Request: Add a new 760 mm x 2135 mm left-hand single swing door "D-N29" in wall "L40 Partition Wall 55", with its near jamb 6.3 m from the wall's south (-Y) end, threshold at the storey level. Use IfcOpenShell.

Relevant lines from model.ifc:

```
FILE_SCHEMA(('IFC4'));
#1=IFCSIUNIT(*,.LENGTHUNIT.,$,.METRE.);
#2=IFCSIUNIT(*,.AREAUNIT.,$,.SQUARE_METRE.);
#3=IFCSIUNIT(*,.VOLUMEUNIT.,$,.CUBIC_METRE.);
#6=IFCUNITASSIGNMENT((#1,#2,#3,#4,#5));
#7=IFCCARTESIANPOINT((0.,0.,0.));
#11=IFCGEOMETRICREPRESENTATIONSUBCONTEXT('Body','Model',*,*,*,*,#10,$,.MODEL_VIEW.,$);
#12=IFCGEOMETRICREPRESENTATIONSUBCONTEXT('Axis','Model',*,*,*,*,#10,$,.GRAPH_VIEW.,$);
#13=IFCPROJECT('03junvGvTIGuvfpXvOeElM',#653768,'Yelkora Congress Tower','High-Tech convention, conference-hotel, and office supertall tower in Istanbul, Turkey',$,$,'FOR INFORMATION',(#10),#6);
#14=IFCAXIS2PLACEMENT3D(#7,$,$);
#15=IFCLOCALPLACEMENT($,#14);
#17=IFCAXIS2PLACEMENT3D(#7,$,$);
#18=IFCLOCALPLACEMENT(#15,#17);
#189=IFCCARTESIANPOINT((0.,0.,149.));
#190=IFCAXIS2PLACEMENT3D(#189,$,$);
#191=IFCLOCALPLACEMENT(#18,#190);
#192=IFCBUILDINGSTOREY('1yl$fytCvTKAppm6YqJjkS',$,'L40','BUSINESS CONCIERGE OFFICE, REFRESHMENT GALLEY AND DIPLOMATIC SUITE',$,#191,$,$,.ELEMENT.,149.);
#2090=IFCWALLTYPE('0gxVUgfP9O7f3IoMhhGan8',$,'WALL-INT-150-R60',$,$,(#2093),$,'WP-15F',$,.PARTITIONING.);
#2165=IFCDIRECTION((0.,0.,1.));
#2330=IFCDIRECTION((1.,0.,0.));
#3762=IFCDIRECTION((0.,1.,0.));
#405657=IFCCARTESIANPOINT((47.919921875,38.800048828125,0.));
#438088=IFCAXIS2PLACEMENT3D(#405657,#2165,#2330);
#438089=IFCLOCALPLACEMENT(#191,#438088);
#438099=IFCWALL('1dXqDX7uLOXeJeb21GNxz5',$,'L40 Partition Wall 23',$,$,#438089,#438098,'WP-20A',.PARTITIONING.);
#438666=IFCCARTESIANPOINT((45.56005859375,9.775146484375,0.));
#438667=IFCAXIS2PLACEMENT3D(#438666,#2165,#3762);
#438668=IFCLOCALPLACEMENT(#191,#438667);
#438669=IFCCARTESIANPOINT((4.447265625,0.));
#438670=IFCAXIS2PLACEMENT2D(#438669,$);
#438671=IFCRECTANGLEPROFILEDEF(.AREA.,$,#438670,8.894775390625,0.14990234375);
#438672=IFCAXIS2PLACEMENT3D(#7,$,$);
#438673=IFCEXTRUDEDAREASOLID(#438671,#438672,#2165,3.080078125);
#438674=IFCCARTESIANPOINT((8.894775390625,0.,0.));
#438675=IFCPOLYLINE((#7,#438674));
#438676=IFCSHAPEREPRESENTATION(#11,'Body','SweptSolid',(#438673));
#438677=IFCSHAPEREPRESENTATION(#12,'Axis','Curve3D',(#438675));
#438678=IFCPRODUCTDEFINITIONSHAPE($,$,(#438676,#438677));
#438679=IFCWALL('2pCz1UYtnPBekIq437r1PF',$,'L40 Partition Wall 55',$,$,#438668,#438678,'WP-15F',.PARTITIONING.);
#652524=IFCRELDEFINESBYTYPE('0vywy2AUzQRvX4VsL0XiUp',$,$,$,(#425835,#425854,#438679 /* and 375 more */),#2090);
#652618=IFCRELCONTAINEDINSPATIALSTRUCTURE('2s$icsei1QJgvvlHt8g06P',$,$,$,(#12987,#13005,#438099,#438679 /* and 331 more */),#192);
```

```python
import numpy as np
import ifcopenshell
import ifcopenshell.api.feature
import ifcopenshell.api.geometry
import ifcopenshell.api.root
import ifcopenshell.api.spatial
import ifcopenshell.geom
import ifcopenshell.util.element
import ifcopenshell.util.placement
import ifcopenshell.util.representation
import ifcopenshell.util.shape
import ifcopenshell.util.unit

model = ifcopenshell.open("model.ifc")
unit_scale = ifcopenshell.util.unit.calculate_unit_scale(model)
settings = ifcopenshell.geom.settings()


def volume(element):
    """Net volume in cubic metres, openings subtracted."""
    shape = ifcopenshell.geom.create_shape(settings, element)
    return ifcopenshell.util.shape.get_volume(shape.geometry)


wall = model.by_guid("2pCz1UYtnPBekIq437r1PF")
storey = ifcopenshell.util.element.get_container(wall, ifc_class="IfcBuildingStorey")
context = ifcopenshell.util.representation.get_context(model, "Model", "Body", "MODEL_VIEW")
before = volume(wall)

width, height, from_end, sill = 0.76, 2.135, 6.3, 0.0  # metres

# The wall runs along its own X axis, and the end named is its -X end.
wall_shape = ifcopenshell.geom.create_shape(settings, wall)
x, y, z = ifcopenshell.util.shape.get_vertices(wall_shape.geometry).T
start = x.min() + from_end
face, thickness = float(y.min()), float(y.max() - y.min())
wall_matrix = ifcopenshell.util.placement.get_local_placement(wall.ObjectPlacement)
level = ifcopenshell.util.placement.get_local_placement(storey.ObjectPlacement)[2, 3]


def in_wall(x, y):
    """Placement at x, y metres in the wall's axes, at sill height."""
    matrix = wall_matrix.copy()
    matrix[:, 3] = wall_matrix @ np.array([x / unit_scale, y / unit_scale, 0.0, 1.0])
    matrix[2, 3] = level + sill / unit_scale
    return matrix


# Opening: a box that overshoots both wall faces by 50 mm.
opening = ifcopenshell.api.root.create_entity(model, ifc_class="IfcOpeningElement", predefined_type="OPENING")
box = ifcopenshell.api.geometry.add_wall_representation(
    model, context=context, length=width, height=height, thickness=thickness + 0.1
)
ifcopenshell.api.geometry.assign_representation(model, product=opening, representation=box)
ifcopenshell.api.geometry.edit_object_placement(model, product=opening, matrix=in_wall(start, face - 0.05), is_si=False)
ifcopenshell.api.feature.add_feature(model, feature=opening, element=wall)

door = ifcopenshell.api.root.create_entity(model, ifc_class="IfcDoor", name="D-N29", predefined_type="DOOR")
door.OverallWidth, door.OverallHeight = width / unit_scale, height / unit_scale
door.OperationType = "SINGLE_SWING_LEFT"
body = ifcopenshell.api.geometry.add_door_representation(
    model,
    context=context,
    overall_width=door.OverallWidth,
    overall_height=door.OverallHeight,
    operation_type="SINGLE_SWING_LEFT",
    lining_properties={"LiningDepth": thickness / unit_scale, "ThresholdDepth": thickness / unit_scale},
)
ifcopenshell.api.geometry.assign_representation(model, product=door, representation=body)
ifcopenshell.api.spatial.assign_container(model, products=[door], relating_structure=storey)
ifcopenshell.api.feature.add_filling(model, opening=opening, element=door)

# The lining spans the wall, so the door starts at the wall face.
ifcopenshell.api.geometry.edit_object_placement(model, product=door, matrix=in_wall(start, face), is_si=False)

after = volume(wall)

print(f"wall volume {before:.3f} -> {after:.3f} m3")

model.write("model_v2.ifc")
```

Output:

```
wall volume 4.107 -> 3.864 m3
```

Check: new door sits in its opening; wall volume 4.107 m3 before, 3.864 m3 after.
